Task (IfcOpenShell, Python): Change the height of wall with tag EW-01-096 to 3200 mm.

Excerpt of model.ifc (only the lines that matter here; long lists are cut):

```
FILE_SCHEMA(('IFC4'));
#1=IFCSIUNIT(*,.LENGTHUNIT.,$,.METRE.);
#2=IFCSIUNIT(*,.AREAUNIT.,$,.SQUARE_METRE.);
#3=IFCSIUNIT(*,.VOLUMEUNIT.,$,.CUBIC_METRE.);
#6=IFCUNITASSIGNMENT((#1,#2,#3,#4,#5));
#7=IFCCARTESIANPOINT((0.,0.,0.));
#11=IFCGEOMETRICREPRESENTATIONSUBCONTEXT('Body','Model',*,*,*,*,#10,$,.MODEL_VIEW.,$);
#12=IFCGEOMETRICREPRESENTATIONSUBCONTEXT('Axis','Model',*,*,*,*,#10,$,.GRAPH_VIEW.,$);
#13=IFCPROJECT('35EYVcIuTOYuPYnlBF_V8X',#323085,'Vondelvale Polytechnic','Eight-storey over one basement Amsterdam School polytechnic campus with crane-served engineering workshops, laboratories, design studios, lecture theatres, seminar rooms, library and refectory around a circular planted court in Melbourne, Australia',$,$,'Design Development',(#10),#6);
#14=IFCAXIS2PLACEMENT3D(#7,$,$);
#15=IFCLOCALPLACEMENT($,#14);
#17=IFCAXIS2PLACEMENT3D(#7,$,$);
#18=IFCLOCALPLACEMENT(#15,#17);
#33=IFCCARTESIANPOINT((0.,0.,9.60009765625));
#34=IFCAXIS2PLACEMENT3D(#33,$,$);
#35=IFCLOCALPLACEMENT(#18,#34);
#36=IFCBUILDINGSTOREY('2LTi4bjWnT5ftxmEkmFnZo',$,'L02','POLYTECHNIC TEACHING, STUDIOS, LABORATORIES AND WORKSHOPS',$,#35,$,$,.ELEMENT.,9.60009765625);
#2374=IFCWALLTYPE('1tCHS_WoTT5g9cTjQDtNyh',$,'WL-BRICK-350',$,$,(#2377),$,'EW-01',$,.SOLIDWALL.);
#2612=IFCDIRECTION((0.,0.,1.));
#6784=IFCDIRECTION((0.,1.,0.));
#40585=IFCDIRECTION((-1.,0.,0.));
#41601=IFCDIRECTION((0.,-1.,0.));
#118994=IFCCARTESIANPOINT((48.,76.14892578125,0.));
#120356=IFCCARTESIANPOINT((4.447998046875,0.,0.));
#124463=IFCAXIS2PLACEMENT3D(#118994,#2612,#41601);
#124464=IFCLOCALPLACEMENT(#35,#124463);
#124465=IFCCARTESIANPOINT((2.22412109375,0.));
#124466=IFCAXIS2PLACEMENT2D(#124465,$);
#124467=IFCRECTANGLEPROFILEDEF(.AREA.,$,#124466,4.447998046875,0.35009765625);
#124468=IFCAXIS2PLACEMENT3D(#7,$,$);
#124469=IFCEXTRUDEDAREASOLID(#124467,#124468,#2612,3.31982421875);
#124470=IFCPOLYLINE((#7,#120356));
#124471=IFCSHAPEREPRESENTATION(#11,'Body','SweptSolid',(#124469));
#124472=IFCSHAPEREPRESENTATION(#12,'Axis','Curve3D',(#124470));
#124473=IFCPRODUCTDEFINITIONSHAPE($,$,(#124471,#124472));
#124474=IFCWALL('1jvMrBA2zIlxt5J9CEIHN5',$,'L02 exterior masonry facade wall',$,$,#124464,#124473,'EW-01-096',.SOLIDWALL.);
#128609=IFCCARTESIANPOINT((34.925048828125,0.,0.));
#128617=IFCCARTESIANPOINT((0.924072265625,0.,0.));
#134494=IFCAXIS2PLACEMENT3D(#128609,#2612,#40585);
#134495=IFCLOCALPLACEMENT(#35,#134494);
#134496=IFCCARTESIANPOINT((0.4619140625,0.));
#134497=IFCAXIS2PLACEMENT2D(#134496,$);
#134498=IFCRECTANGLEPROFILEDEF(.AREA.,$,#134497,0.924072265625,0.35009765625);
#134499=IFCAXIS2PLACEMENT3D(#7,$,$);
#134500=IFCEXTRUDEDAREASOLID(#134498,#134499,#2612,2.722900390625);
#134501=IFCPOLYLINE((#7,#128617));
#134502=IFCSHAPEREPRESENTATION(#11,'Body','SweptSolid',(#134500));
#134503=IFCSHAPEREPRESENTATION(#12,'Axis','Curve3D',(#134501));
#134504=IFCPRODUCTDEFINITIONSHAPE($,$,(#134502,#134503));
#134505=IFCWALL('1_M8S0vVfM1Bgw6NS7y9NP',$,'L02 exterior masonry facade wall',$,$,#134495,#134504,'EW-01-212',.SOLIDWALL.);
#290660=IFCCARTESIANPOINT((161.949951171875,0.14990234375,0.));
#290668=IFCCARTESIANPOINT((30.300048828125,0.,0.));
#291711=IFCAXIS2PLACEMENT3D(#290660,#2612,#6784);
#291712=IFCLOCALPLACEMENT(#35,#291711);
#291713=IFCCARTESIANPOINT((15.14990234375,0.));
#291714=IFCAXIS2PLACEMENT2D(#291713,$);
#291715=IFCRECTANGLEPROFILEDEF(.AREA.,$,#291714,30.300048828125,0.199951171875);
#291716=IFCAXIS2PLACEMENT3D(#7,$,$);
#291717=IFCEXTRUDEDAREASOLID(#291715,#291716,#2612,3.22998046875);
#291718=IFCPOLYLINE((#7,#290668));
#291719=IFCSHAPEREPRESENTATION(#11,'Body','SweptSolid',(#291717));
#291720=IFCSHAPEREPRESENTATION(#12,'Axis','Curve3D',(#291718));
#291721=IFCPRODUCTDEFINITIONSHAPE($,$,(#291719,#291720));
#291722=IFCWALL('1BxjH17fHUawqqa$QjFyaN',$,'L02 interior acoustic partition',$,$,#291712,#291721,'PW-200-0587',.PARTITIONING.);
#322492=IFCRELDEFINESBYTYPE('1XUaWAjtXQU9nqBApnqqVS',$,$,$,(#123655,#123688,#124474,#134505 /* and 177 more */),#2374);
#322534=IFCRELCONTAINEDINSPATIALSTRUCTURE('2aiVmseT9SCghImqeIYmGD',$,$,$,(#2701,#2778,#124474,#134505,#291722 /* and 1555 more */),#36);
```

```python
import ifcopenshell
import ifcopenshell.geom
import ifcopenshell.util.representation
import ifcopenshell.util.shape
import ifcopenshell.util.unit

model = ifcopenshell.open("model.ifc")
unit_scale = ifcopenshell.util.unit.calculate_unit_scale(model)
settings = ifcopenshell.geom.settings()


def volume(element):
    """Net volume in cubic metres, openings subtracted."""
    shape = ifcopenshell.geom.create_shape(settings, element)
    return ifcopenshell.util.shape.get_volume(shape.geometry)


wall = model.by_id(124474)
before = volume(wall)

body = ifcopenshell.util.representation.get_representation(wall, "Model", "Body")
solid = body.Items[0]
old_height = solid.Depth
solid.Depth = 3.2 / unit_scale
after = volume(wall)

print(f"height {old_height:g} -> {solid.Depth:g}, volume {before:.3f} -> {after:.3f} m3")

model.write("model_v2.ifc")
```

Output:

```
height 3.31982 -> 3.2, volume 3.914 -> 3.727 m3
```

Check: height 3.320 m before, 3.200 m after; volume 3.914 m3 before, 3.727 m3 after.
